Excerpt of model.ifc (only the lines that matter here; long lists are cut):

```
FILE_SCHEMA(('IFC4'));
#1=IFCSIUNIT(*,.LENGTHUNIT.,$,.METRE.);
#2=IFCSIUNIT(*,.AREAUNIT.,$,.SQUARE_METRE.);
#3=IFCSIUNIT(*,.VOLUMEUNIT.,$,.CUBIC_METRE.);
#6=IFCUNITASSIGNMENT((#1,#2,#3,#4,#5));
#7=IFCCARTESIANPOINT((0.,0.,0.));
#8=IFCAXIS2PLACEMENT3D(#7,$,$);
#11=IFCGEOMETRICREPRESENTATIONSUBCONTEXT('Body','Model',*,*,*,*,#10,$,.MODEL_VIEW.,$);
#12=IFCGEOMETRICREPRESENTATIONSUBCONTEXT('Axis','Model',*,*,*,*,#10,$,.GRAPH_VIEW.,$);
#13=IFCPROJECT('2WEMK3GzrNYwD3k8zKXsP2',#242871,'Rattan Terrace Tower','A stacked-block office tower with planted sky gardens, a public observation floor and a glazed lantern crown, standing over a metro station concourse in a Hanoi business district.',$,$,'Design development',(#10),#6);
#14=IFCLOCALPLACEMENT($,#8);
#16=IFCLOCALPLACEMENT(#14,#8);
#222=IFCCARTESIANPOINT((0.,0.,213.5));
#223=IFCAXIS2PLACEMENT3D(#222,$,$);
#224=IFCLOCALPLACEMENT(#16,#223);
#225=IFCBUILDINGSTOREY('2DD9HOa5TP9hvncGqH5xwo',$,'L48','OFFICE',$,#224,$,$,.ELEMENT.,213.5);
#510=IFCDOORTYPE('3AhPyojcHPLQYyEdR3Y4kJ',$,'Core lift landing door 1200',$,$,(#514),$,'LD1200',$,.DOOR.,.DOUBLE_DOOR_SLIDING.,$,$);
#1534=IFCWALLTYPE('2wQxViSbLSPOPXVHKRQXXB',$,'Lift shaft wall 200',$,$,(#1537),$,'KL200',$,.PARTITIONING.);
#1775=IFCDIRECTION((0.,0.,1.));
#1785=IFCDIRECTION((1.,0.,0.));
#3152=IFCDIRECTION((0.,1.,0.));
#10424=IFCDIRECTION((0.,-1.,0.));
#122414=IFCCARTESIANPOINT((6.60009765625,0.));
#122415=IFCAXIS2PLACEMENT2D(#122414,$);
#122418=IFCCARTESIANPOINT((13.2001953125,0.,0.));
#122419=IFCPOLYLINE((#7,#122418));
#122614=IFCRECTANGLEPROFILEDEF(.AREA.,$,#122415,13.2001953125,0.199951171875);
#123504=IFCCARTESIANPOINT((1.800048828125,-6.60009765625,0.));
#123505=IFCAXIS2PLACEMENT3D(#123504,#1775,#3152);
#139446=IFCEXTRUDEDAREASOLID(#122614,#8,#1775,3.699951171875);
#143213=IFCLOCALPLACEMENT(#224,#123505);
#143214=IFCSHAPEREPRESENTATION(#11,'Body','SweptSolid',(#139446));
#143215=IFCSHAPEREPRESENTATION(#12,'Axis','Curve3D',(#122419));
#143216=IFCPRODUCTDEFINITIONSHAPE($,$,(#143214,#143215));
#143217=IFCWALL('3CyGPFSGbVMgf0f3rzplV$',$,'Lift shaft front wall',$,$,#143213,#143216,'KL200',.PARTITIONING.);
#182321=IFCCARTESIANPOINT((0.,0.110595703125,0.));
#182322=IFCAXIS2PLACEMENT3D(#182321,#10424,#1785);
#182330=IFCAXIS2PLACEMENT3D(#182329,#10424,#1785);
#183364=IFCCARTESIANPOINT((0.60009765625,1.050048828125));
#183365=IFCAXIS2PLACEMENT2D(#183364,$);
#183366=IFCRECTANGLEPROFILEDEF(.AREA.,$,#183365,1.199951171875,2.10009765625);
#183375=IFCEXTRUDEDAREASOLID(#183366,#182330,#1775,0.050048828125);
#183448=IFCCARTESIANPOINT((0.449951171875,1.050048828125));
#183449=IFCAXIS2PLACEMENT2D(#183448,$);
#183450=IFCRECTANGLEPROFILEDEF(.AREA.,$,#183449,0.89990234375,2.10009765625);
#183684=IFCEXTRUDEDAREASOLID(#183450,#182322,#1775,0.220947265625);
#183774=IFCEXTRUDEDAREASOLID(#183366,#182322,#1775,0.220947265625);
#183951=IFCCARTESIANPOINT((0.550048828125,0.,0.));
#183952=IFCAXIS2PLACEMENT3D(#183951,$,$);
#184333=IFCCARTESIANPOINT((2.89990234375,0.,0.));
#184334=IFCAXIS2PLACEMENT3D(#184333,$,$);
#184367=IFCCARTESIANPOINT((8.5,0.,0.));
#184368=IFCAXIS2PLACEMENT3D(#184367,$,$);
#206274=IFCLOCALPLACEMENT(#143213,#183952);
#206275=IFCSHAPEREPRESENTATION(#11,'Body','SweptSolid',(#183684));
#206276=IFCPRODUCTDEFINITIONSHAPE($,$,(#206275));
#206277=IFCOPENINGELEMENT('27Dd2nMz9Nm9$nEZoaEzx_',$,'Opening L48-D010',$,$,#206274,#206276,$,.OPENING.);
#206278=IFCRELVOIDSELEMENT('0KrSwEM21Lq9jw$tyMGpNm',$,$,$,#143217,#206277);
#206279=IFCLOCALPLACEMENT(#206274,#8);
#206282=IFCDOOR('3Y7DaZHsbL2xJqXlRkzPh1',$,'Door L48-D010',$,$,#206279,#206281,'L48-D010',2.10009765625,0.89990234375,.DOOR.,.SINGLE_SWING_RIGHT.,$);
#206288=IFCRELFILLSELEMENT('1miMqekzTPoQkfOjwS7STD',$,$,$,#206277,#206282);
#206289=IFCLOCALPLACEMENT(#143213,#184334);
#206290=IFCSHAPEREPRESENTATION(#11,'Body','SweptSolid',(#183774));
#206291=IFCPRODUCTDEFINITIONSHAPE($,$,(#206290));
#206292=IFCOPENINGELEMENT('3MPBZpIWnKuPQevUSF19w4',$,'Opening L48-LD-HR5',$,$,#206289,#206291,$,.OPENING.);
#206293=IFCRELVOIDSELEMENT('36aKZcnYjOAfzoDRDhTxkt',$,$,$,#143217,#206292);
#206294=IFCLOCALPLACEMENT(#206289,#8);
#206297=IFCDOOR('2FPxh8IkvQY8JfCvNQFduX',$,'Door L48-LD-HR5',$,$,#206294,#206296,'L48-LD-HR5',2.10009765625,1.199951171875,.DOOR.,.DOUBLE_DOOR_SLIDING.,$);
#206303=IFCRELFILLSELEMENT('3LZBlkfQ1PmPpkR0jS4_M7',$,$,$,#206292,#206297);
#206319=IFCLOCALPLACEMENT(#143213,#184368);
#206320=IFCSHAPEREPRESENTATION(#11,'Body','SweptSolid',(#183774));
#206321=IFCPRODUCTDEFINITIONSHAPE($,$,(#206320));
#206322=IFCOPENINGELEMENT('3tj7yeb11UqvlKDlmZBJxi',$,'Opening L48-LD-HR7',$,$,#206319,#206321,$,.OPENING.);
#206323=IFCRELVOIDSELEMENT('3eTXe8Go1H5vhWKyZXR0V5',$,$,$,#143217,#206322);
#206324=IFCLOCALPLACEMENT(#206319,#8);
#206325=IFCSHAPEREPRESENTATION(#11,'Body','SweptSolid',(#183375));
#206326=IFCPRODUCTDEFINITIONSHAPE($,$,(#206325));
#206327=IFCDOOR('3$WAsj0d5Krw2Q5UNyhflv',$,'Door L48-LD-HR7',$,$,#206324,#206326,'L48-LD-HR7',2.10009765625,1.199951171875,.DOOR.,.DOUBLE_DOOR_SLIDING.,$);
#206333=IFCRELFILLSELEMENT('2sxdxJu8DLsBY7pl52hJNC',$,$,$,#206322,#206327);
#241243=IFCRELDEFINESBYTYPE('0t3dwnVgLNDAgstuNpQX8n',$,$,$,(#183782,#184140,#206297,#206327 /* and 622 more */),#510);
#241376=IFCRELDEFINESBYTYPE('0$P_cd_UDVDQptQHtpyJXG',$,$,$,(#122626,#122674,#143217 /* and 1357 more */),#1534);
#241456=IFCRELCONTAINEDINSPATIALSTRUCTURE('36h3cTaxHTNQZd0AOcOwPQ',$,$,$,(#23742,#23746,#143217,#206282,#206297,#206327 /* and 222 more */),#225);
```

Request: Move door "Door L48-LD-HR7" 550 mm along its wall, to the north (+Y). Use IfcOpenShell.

```python
import ifcopenshell
import ifcopenshell.api.geometry
import ifcopenshell.util.placement
import ifcopenshell.util.unit

model = ifcopenshell.open("model.ifc")
unit_scale = ifcopenshell.util.unit.calculate_unit_scale(model)

door = model.by_guid("3$WAsj0d5Krw2Q5UNyhflv")
opening = door.FillsVoids[0].RelatingOpeningElement
wall = opening.VoidsElements[0].RelatingBuildingElement

wall_matrix = ifcopenshell.util.placement.get_local_placement(wall.ObjectPlacement)
shift = wall_matrix[:3, 0] * 0.55 / unit_scale
before = ifcopenshell.util.placement.get_local_placement(door.ObjectPlacement)[:3, 3].copy()

# The door is placed relative to its opening, so it follows when the opening moves.
matrix = ifcopenshell.util.placement.get_local_placement(opening.ObjectPlacement)
matrix[:3, 3] += shift
ifcopenshell.api.geometry.edit_object_placement(
    model, product=opening, matrix=matrix, is_si=False, should_transform_children=True
)

after = ifcopenshell.util.placement.get_local_placement(door.ObjectPlacement)[:3, 3]
print("door moved by", (after - before).round(3) + 0.0)

model.write("model_rev.ifc")
```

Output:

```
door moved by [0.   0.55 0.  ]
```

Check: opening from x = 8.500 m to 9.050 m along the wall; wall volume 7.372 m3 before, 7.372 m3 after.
